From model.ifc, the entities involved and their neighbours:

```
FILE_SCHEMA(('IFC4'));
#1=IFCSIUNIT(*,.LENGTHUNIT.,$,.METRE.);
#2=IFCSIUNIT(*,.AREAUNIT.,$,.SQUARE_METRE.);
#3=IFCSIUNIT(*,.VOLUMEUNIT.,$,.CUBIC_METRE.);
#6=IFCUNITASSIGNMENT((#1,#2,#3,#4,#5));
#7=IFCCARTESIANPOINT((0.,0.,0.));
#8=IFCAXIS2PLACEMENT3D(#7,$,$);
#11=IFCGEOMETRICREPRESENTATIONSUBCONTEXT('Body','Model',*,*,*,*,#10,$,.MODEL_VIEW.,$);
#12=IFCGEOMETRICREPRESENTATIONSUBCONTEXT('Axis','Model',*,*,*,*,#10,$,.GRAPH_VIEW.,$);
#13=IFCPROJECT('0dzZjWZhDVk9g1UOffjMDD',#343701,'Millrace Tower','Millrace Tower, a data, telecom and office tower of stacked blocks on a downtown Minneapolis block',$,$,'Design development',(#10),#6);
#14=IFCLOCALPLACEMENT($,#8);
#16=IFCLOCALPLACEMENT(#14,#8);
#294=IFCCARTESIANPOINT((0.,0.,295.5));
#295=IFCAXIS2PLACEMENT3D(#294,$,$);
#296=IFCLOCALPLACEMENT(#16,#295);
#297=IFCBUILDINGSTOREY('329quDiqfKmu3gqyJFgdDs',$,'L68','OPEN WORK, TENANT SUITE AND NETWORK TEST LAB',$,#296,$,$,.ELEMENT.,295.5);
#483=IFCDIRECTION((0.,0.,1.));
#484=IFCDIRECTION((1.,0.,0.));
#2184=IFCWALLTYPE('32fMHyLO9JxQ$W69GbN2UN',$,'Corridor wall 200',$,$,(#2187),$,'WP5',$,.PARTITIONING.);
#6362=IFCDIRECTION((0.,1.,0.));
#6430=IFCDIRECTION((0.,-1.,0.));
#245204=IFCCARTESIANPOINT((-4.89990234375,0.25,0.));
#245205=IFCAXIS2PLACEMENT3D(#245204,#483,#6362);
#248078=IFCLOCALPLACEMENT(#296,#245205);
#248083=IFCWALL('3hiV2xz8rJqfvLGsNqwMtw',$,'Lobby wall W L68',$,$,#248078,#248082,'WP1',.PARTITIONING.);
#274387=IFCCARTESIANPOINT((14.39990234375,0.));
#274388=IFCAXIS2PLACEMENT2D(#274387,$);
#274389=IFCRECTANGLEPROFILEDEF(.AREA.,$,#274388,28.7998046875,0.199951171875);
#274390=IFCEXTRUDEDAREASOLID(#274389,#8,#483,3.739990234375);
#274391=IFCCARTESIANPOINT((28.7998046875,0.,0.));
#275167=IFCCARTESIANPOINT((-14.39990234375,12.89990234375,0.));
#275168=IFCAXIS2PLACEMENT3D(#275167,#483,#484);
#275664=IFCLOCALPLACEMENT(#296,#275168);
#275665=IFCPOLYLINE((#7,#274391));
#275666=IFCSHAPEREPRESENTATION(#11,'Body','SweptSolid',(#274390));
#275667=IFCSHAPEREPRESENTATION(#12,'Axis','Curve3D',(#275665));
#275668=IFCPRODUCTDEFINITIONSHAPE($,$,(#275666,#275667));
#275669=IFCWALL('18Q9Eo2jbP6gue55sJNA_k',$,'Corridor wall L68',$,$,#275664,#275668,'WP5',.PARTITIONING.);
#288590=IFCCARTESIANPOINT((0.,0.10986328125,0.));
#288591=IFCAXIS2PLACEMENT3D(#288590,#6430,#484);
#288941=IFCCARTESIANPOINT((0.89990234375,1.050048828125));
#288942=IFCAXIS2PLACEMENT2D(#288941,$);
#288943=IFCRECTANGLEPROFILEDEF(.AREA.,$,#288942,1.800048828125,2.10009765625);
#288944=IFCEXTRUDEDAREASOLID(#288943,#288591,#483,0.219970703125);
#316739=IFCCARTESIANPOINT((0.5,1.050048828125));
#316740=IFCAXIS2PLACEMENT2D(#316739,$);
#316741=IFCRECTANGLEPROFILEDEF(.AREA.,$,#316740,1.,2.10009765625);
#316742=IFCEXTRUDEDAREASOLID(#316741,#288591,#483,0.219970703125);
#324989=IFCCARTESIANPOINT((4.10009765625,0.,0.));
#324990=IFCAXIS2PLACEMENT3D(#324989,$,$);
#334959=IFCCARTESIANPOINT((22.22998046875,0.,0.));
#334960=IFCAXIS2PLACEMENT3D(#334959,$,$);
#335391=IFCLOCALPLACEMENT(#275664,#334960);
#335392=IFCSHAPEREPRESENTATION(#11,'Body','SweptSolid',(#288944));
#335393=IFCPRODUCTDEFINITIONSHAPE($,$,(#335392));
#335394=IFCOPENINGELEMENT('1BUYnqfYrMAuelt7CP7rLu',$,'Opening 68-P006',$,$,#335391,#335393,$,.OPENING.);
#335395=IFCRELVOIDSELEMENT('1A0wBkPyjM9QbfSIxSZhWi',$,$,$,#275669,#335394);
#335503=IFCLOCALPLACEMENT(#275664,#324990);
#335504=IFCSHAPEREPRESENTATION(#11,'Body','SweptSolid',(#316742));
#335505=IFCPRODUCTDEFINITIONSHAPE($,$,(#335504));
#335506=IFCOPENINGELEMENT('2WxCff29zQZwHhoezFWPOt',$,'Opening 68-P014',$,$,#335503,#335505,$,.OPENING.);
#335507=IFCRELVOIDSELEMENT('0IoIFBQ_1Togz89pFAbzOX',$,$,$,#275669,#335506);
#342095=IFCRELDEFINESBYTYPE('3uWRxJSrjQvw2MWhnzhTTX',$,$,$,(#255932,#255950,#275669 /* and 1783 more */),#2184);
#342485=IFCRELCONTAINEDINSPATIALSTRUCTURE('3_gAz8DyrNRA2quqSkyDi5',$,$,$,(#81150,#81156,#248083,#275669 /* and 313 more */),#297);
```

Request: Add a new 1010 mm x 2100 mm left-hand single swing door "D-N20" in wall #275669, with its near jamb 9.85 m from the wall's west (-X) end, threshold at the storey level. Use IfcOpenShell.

```python
import numpy as np
import ifcopenshell
import ifcopenshell.api.feature
import ifcopenshell.api.geometry
import ifcopenshell.api.root
import ifcopenshell.api.spatial
import ifcopenshell.geom
import ifcopenshell.util.element
import ifcopenshell.util.placement
import ifcopenshell.util.representation
import ifcopenshell.util.shape
import ifcopenshell.util.unit

model = ifcopenshell.open("model.ifc")
unit_scale = ifcopenshell.util.unit.calculate_unit_scale(model)
settings = ifcopenshell.geom.settings()


def volume(element):
    """Net volume in cubic metres, openings subtracted."""
    shape = ifcopenshell.geom.create_shape(settings, element)
    return ifcopenshell.util.shape.get_volume(shape.geometry)


wall = model.by_guid("18Q9Eo2jbP6gue55sJNA_k")
storey = ifcopenshell.util.element.get_container(wall, ifc_class="IfcBuildingStorey")
context = ifcopenshell.util.representation.get_context(model, "Model", "Body", "MODEL_VIEW")
before = volume(wall)

width, height, from_end, sill = 1.01, 2.1, 9.85, 0.0  # metres

# The wall runs along its own X axis, and the end named is its -X end.
wall_shape = ifcopenshell.geom.create_shape(settings, wall)
x, y, z = ifcopenshell.util.shape.get_vertices(wall_shape.geometry).T
start = x.min() + from_end
face, thickness = float(y.min()), float(y.max() - y.min())
wall_matrix = ifcopenshell.util.placement.get_local_placement(wall.ObjectPlacement)
level = ifcopenshell.util.placement.get_local_placement(storey.ObjectPlacement)[2, 3]


def in_wall(x, y):
    """Placement at x, y metres in the wall's axes, at sill height."""
    matrix = wall_matrix.copy()
    matrix[:, 3] = wall_matrix @ np.array([x / unit_scale, y / unit_scale, 0.0, 1.0])
    matrix[2, 3] = level + sill / unit_scale
    return matrix


# Opening: a box that overshoots both wall faces by 50 mm.
opening = ifcopenshell.api.root.create_entity(model, ifc_class="IfcOpeningElement", predefined_type="OPENING")
box = ifcopenshell.api.geometry.add_wall_representation(
    model, context=context, length=width, height=height, thickness=thickness + 0.1
)
ifcopenshell.api.geometry.assign_representation(model, product=opening, representation=box)
ifcopenshell.api.geometry.edit_object_placement(model, product=opening, matrix=in_wall(start, face - 0.05), is_si=False)
ifcopenshell.api.feature.add_feature(model, feature=opening, element=wall)

door = ifcopenshell.api.root.create_entity(model, ifc_class="IfcDoor", name="D-N20", predefined_type="DOOR")
door.OverallWidth, door.OverallHeight = width / unit_scale, height / unit_scale
door.OperationType = "SINGLE_SWING_LEFT"
body = ifcopenshell.api.geometry.add_door_representation(
    model,
    context=context,
    overall_width=door.OverallWidth,
    overall_height=door.OverallHeight,
    operation_type="SINGLE_SWING_LEFT",
    lining_properties={"LiningDepth": thickness / unit_scale, "ThresholdDepth": thickness / unit_scale},
)
ifcopenshell.api.geometry.assign_representation(model, product=door, representation=body)
ifcopenshell.api.spatial.assign_container(model, products=[door], relating_structure=storey)
ifcopenshell.api.feature.add_filling(model, opening=opening, element=door)

# The lining spans the wall, so the door starts at the wall face.
ifcopenshell.api.geometry.edit_object_placement(model, product=door, matrix=in_wall(start, face), is_si=False)

after = volume(wall)

print(f"wall volume {before:.3f} -> {after:.3f} m3")

model.write("model_rev.ifc")
```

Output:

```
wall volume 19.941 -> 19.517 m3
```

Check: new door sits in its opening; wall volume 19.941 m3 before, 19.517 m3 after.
